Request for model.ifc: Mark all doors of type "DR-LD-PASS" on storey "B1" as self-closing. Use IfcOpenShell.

First a look at what the model holds.

```python
import ifcopenshell
import ifcopenshell.util.element

model = ifcopenshell.open("model.ifc")
print(model.schema)
storey = next(s for s in model.by_type("IfcBuildingStorey") if s.Name == "B1")
doors = [e for e in ifcopenshell.util.element.get_decomposition(storey) if e.is_a("IfcDoor")]
seen = {}
for e in doors:
    element_type = ifcopenshell.util.element.get_type(e)
    key = (element_type.Name if element_type != e and element_type else None, ifcopenshell.util.element.get_pset(e, "Pset_DoorCommon", "SelfClosing"))
    seen[key] = seen.get(key, 0) + 1
for (name, value), count in sorted(seen.items(), key=str):
    print(count, "x", name, "|", value)
```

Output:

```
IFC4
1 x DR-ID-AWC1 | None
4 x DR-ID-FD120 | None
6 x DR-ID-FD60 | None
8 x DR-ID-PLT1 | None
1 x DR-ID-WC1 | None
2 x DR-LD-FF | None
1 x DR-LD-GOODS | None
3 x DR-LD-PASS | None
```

```python
import ifcopenshell
import ifcopenshell.api.pset
import ifcopenshell.util.element

model = ifcopenshell.open("model.ifc")

storey = next(s for s in model.by_type("IfcBuildingStorey") if s.Name == "B1")
doors = [e for e in ifcopenshell.util.element.get_decomposition(storey) if e.is_a("IfcDoor")]

count = 0
for e in doors:
    element_type = ifcopenshell.util.element.get_type(e)
    if element_type in (None, e) or element_type.Name != "DR-LD-PASS":
        continue
    # add_pset returns the element's existing set when there is one.
    pset = ifcopenshell.api.pset.add_pset(model, product=e, name="Pset_DoorCommon")
    ifcopenshell.api.pset.edit_pset(model, pset=pset, properties={"SelfClosing": True})
    count += 1

print(count, "doors updated")

model.write("model_updated.ifc")
```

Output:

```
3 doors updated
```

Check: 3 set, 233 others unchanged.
